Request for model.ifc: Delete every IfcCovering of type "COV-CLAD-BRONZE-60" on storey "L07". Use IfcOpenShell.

First a look at what the model holds.

```python
import ifcopenshell
import ifcopenshell.util.element

model = ifcopenshell.open("model.ifc")
print(model.schema)
storey = next(s for s in model.by_type("IfcBuildingStorey") if s.Name == "L07")
coverings = [e for e in ifcopenshell.util.element.get_decomposition(storey) if e.is_a("IfcCovering")]
seen = {}
for e in coverings:
    element_type = ifcopenshell.util.element.get_type(e)
    name = element_type.Name if element_type not in (None, e) else None
    seen[name] = seen.get(name, 0) + 1
for name, count in sorted(seen.items(), key=str):
    print(count, "x", name)
```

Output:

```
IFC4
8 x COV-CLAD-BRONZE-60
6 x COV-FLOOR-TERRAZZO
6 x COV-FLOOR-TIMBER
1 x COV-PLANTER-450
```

```python
import ifcopenshell
import ifcopenshell.api.root
import ifcopenshell.util.element

model = ifcopenshell.open("model.ifc")

storey = next(s for s in model.by_type("IfcBuildingStorey") if s.Name == "L07")
coverings = [e for e in ifcopenshell.util.element.get_decomposition(storey) if e.is_a("IfcCovering")]
targets = [e for e in coverings if (t := ifcopenshell.util.element.get_type(e)) not in (None, e) and t.Name == "COV-CLAD-BRONZE-60"]

for e in targets:
    ifcopenshell.api.root.remove_product(model, product=e)
print(len(targets), "removed")

model.write("model_edited.ifc")
```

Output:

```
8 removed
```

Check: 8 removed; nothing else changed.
